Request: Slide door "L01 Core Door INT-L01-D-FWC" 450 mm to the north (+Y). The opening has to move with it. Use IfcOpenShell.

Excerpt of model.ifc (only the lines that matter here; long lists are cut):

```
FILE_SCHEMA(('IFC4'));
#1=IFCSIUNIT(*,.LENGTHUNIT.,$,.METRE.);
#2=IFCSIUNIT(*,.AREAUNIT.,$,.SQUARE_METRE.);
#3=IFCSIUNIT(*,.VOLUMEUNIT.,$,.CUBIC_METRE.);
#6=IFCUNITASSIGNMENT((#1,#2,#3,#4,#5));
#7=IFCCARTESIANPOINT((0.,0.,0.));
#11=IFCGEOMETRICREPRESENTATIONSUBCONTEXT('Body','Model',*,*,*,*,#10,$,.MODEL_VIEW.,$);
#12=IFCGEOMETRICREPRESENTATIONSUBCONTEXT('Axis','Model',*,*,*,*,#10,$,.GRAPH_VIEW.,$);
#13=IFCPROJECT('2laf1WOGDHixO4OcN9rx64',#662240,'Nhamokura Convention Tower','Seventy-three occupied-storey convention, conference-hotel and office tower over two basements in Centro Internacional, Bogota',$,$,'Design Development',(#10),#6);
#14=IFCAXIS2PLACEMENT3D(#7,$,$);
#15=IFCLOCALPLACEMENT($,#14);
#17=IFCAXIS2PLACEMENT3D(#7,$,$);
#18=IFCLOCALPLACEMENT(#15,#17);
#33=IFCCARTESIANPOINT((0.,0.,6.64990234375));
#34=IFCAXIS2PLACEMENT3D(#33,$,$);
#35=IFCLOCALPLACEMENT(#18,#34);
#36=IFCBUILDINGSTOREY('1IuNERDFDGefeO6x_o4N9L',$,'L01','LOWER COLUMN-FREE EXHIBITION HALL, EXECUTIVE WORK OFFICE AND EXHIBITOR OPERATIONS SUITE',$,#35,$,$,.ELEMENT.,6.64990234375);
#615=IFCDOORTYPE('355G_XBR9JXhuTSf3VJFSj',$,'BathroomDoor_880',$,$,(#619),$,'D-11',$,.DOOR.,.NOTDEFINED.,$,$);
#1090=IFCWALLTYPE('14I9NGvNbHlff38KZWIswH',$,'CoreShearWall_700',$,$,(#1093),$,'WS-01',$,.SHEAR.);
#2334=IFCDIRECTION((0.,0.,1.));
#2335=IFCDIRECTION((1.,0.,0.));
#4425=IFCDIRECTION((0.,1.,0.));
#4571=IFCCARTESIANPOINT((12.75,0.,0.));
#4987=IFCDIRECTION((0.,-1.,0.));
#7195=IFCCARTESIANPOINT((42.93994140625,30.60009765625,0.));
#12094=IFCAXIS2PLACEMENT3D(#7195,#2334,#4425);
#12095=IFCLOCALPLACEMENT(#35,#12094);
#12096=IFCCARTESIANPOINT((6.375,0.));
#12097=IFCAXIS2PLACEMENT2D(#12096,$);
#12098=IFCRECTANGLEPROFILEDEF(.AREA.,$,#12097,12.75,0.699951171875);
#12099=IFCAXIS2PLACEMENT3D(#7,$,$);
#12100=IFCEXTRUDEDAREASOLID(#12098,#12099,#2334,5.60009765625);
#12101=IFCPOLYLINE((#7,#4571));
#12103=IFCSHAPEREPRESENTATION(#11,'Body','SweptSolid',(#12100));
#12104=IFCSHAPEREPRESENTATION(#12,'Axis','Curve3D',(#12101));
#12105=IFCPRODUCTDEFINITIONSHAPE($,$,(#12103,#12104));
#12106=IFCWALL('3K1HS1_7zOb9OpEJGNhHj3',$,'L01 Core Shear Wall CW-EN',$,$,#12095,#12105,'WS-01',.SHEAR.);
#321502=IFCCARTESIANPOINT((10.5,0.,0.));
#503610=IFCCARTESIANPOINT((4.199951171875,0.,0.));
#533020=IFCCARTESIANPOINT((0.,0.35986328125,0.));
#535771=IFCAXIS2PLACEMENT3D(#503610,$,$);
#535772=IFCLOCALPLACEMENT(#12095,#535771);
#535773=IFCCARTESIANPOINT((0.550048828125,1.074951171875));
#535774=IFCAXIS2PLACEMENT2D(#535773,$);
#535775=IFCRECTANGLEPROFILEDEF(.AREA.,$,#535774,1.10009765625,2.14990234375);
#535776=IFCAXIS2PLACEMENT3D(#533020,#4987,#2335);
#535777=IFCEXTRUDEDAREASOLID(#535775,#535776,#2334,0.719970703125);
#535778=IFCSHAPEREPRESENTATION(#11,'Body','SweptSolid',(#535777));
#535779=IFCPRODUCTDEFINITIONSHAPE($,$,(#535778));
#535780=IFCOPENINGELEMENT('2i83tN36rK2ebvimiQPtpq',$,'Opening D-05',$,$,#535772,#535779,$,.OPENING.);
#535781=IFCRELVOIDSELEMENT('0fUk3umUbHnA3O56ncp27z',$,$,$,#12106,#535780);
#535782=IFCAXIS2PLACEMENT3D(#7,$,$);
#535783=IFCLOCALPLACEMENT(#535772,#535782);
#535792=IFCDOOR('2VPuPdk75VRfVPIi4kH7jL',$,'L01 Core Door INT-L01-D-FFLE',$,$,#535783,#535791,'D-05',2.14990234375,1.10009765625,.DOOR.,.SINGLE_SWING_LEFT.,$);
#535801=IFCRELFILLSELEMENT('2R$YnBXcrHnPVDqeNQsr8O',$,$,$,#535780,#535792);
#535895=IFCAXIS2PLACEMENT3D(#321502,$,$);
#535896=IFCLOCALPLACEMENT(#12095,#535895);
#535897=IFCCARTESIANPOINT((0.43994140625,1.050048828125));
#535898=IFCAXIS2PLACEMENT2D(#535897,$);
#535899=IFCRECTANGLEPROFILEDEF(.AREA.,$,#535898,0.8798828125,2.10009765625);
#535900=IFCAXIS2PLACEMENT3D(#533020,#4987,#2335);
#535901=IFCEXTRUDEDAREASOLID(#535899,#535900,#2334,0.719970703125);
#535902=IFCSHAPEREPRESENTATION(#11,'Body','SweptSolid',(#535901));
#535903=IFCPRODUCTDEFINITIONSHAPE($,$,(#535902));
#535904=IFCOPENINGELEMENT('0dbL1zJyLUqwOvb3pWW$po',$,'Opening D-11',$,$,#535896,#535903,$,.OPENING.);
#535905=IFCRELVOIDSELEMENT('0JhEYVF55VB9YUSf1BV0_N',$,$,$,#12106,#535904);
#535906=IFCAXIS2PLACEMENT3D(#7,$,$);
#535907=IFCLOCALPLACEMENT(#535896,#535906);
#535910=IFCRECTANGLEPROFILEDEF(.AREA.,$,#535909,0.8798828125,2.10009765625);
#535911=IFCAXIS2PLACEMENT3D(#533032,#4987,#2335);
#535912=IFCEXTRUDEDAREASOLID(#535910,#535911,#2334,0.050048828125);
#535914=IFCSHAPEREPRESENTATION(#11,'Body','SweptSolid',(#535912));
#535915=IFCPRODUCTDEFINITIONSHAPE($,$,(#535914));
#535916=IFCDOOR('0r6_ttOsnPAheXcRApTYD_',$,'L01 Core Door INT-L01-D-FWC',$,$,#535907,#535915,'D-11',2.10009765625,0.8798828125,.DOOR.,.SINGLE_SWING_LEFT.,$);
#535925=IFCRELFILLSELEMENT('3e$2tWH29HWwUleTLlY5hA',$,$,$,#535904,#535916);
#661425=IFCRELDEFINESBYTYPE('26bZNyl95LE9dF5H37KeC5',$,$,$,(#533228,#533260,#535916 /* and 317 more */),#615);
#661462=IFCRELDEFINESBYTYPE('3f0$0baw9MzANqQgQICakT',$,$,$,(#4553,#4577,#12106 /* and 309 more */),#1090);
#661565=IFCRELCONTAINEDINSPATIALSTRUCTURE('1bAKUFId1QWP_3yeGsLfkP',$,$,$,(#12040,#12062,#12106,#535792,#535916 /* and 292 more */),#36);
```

```python
import ifcopenshell
import ifcopenshell.api.geometry
import ifcopenshell.util.placement

model = ifcopenshell.open("model.ifc")

door = model.by_id(535916)
opening = door.FillsVoids[0].RelatingOpeningElement
wall = opening.VoidsElements[0].RelatingBuildingElement

wall_matrix = ifcopenshell.util.placement.get_local_placement(wall.ObjectPlacement)
shift = wall_matrix[:3, 0] * 0.45
before = ifcopenshell.util.placement.get_local_placement(door.ObjectPlacement)[:3, 3].copy()

# The door is placed relative to its opening, so it follows when the opening moves.
matrix = ifcopenshell.util.placement.get_local_placement(opening.ObjectPlacement)
matrix[:3, 3] += shift
ifcopenshell.api.geometry.edit_object_placement(
    model, product=opening, matrix=matrix, is_si=False, should_transform_children=True
)

after = ifcopenshell.util.placement.get_local_placement(door.ObjectPlacement)[:3, 3]
print("door moved by", (after - before).round(3) + 0.0)

model.write("model_rev.ifc")
```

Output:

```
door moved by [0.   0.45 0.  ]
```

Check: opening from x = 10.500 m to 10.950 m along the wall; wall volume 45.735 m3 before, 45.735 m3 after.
